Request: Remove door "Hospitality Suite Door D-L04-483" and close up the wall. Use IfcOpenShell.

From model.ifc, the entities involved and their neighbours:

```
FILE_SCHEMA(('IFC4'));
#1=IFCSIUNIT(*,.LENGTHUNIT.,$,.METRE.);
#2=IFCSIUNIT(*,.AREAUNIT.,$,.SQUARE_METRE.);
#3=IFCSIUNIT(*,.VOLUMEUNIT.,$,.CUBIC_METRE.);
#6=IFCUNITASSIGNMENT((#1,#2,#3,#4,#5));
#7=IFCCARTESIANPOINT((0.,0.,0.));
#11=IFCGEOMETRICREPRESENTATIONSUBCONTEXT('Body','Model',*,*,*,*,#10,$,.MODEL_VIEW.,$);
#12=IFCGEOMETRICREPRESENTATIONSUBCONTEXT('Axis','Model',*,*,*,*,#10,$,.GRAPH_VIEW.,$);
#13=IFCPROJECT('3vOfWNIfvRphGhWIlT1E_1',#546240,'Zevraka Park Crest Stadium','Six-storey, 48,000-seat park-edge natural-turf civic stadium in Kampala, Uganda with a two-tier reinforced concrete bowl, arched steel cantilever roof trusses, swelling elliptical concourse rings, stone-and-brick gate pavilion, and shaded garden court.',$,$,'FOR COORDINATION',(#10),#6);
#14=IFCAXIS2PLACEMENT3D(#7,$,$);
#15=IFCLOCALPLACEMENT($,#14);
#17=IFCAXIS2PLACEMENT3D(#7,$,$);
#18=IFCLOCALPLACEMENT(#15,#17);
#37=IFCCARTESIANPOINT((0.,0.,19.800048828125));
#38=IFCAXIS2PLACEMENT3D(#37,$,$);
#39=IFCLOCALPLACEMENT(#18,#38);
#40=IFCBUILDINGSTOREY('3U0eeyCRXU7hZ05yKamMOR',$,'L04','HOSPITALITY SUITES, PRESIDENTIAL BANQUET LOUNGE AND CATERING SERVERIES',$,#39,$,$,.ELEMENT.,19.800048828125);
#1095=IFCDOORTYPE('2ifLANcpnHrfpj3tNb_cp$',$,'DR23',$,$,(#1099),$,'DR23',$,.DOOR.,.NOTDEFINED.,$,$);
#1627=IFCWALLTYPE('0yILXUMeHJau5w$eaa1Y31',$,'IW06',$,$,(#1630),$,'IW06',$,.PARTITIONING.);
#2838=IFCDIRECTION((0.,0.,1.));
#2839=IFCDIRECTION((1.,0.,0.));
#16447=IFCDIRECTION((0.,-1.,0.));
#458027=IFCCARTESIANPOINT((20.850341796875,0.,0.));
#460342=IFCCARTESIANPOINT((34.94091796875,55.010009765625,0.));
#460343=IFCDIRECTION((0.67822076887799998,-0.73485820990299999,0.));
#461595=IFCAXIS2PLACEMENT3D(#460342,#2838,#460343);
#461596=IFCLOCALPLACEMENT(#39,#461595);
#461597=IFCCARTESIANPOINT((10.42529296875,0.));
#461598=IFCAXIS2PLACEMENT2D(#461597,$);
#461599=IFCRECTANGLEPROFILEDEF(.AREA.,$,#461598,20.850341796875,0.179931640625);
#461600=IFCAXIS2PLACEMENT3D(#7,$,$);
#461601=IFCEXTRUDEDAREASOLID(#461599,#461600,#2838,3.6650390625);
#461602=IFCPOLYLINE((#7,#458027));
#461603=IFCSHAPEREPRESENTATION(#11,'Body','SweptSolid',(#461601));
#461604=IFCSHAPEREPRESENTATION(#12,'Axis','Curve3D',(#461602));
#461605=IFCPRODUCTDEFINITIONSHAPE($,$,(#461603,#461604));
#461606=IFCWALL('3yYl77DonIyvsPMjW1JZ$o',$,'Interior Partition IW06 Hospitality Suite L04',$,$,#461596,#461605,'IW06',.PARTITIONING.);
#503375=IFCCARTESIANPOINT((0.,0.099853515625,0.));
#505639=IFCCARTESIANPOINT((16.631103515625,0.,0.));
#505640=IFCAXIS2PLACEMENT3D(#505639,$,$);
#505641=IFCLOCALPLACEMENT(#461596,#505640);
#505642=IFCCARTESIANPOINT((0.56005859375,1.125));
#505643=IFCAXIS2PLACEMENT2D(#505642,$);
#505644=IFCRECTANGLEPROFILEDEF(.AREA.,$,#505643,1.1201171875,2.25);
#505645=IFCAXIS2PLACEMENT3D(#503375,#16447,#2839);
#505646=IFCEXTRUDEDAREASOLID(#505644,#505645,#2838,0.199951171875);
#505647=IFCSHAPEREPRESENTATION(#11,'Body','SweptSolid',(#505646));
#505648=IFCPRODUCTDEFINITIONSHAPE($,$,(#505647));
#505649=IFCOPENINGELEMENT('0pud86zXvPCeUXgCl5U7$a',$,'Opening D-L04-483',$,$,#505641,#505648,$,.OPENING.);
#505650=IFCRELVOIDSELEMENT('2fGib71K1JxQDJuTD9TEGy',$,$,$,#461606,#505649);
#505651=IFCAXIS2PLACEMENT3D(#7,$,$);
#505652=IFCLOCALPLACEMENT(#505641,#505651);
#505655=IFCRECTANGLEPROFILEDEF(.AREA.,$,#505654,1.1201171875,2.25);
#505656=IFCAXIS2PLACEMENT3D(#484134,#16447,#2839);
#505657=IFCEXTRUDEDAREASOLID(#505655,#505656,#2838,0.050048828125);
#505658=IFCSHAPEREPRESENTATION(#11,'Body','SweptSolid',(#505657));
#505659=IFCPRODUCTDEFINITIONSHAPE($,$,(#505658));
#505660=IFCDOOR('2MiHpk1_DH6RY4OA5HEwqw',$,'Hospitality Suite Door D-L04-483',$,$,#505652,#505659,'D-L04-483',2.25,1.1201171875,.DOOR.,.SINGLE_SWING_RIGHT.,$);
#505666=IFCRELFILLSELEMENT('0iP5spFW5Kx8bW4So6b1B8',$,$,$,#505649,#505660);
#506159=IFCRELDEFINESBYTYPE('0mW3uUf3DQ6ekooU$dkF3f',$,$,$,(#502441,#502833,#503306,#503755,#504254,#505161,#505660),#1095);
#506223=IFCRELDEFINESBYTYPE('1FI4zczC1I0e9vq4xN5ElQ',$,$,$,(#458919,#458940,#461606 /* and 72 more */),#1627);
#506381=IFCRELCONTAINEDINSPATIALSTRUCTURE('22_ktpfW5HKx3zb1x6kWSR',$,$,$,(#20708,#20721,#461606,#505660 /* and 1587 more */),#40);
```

```python
import ifcopenshell
import ifcopenshell.api.feature
import ifcopenshell.api.root
import ifcopenshell.geom
import ifcopenshell.util.shape

model = ifcopenshell.open("model.ifc")
settings = ifcopenshell.geom.settings()


def volume(element):
    """Net volume in cubic metres, openings subtracted."""
    shape = ifcopenshell.geom.create_shape(settings, element)
    return ifcopenshell.util.shape.get_volume(shape.geometry)


door = model.by_guid("2MiHpk1_DH6RY4OA5HEwqw")
opening = door.FillsVoids[0].RelatingOpeningElement
wall = opening.VoidsElements[0].RelatingBuildingElement
before = volume(wall)

ifcopenshell.api.root.remove_product(model, product=door)
ifcopenshell.api.feature.remove_feature(model, feature=opening)

after = volume(wall)

print(f"wall volume {before:.3f} -> {after:.3f} m3")

model.write("model_v2.ifc")
```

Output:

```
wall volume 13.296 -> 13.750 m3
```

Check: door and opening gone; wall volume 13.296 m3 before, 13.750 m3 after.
